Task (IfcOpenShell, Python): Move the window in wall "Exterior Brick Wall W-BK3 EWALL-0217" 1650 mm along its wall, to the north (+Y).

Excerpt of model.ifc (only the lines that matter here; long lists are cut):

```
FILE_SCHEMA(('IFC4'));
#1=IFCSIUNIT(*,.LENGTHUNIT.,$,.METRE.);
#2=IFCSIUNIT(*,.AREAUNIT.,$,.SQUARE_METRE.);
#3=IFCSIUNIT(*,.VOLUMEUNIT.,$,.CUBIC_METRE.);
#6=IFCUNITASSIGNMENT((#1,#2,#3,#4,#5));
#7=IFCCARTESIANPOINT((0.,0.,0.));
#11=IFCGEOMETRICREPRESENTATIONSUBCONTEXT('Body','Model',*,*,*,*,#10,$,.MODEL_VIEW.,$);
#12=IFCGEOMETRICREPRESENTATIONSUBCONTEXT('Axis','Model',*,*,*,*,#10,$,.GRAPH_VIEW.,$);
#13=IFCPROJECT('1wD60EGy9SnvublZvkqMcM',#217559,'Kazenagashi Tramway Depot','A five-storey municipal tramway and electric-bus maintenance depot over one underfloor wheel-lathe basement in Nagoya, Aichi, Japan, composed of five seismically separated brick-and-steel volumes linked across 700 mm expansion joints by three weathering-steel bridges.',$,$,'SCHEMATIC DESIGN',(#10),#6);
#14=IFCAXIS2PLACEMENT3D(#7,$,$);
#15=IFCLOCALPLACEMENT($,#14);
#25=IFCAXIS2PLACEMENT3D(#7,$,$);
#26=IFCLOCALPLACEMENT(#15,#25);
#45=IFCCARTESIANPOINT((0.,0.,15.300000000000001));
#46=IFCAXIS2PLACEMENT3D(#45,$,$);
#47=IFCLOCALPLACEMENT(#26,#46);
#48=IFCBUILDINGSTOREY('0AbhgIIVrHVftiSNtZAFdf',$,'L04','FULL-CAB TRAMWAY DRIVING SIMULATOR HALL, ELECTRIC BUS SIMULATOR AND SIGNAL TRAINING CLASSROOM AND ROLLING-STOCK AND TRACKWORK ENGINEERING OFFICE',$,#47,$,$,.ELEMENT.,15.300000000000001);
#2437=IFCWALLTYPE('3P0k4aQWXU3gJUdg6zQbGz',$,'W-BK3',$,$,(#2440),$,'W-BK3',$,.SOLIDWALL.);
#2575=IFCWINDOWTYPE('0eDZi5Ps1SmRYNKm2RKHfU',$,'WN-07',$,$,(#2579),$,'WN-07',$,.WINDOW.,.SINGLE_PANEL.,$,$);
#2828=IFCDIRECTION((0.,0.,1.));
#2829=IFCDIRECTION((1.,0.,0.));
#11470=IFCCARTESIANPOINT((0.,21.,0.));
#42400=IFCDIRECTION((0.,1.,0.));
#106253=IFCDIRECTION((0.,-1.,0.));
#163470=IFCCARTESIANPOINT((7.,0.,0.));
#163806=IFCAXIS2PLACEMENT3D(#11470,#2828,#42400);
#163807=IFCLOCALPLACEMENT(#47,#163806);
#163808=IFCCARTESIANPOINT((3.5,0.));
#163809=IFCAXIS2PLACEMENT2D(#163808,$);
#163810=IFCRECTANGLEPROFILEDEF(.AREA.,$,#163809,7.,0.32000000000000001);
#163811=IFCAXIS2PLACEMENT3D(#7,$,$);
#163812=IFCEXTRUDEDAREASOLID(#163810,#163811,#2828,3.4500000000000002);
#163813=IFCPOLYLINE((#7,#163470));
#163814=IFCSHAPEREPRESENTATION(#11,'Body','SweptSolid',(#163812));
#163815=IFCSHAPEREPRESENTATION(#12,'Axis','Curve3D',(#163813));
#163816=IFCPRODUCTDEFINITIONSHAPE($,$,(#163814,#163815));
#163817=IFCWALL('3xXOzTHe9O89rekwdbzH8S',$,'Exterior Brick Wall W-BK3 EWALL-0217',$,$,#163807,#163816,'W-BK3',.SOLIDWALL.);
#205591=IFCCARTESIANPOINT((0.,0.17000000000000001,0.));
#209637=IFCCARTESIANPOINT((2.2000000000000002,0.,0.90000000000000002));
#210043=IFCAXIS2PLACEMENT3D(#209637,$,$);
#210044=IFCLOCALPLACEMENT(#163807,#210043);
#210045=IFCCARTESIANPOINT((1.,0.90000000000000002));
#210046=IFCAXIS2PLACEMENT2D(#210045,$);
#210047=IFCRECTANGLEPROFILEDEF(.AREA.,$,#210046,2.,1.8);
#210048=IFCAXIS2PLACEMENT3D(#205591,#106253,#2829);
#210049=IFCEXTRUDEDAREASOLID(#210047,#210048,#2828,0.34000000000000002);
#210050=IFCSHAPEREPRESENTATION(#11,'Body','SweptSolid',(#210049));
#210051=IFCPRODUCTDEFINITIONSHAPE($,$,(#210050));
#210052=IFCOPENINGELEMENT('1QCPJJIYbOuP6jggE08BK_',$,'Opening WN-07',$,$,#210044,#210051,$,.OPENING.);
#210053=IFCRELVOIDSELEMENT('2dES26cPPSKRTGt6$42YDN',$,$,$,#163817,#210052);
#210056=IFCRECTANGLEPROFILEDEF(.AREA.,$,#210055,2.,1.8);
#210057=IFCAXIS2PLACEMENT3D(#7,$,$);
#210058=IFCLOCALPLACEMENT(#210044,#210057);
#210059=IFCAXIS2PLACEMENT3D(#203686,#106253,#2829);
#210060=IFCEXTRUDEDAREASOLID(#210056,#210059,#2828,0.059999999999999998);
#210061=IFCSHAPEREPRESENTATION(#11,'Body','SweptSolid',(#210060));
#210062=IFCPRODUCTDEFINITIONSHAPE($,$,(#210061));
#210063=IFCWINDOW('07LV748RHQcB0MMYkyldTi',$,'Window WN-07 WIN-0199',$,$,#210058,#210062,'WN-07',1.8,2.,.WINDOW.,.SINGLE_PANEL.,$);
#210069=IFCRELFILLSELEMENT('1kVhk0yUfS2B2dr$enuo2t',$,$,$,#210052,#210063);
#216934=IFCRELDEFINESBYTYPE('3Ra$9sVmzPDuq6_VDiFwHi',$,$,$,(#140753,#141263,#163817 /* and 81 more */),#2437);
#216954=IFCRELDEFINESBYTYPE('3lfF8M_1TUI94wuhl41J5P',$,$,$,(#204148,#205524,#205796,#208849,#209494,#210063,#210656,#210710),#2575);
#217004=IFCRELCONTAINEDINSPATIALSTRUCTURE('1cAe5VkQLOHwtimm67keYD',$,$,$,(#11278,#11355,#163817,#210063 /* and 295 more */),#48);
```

```python
import ifcopenshell
import ifcopenshell.api.geometry
import ifcopenshell.util.placement
import ifcopenshell.util.unit

model = ifcopenshell.open("model.ifc")
unit_scale = ifcopenshell.util.unit.calculate_unit_scale(model)

window = model.by_guid("07LV748RHQcB0MMYkyldTi")
opening = window.FillsVoids[0].RelatingOpeningElement
wall = opening.VoidsElements[0].RelatingBuildingElement

wall_matrix = ifcopenshell.util.placement.get_local_placement(wall.ObjectPlacement)
shift = wall_matrix[:3, 0] * 1.65 / unit_scale
before = ifcopenshell.util.placement.get_local_placement(window.ObjectPlacement)[:3, 3].copy()

# The window is placed relative to its opening, so it follows when the opening moves.
matrix = ifcopenshell.util.placement.get_local_placement(opening.ObjectPlacement)
matrix[:3, 3] += shift
ifcopenshell.api.geometry.edit_object_placement(
    model, product=opening, matrix=matrix, is_si=False, should_transform_children=True
)

after = ifcopenshell.util.placement.get_local_placement(window.ObjectPlacement)[:3, 3]
print("window moved by", (after - before).round(3) + 0.0)

model.write("model_v2.ifc")
```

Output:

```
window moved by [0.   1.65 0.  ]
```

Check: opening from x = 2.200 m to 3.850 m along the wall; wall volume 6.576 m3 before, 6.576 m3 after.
